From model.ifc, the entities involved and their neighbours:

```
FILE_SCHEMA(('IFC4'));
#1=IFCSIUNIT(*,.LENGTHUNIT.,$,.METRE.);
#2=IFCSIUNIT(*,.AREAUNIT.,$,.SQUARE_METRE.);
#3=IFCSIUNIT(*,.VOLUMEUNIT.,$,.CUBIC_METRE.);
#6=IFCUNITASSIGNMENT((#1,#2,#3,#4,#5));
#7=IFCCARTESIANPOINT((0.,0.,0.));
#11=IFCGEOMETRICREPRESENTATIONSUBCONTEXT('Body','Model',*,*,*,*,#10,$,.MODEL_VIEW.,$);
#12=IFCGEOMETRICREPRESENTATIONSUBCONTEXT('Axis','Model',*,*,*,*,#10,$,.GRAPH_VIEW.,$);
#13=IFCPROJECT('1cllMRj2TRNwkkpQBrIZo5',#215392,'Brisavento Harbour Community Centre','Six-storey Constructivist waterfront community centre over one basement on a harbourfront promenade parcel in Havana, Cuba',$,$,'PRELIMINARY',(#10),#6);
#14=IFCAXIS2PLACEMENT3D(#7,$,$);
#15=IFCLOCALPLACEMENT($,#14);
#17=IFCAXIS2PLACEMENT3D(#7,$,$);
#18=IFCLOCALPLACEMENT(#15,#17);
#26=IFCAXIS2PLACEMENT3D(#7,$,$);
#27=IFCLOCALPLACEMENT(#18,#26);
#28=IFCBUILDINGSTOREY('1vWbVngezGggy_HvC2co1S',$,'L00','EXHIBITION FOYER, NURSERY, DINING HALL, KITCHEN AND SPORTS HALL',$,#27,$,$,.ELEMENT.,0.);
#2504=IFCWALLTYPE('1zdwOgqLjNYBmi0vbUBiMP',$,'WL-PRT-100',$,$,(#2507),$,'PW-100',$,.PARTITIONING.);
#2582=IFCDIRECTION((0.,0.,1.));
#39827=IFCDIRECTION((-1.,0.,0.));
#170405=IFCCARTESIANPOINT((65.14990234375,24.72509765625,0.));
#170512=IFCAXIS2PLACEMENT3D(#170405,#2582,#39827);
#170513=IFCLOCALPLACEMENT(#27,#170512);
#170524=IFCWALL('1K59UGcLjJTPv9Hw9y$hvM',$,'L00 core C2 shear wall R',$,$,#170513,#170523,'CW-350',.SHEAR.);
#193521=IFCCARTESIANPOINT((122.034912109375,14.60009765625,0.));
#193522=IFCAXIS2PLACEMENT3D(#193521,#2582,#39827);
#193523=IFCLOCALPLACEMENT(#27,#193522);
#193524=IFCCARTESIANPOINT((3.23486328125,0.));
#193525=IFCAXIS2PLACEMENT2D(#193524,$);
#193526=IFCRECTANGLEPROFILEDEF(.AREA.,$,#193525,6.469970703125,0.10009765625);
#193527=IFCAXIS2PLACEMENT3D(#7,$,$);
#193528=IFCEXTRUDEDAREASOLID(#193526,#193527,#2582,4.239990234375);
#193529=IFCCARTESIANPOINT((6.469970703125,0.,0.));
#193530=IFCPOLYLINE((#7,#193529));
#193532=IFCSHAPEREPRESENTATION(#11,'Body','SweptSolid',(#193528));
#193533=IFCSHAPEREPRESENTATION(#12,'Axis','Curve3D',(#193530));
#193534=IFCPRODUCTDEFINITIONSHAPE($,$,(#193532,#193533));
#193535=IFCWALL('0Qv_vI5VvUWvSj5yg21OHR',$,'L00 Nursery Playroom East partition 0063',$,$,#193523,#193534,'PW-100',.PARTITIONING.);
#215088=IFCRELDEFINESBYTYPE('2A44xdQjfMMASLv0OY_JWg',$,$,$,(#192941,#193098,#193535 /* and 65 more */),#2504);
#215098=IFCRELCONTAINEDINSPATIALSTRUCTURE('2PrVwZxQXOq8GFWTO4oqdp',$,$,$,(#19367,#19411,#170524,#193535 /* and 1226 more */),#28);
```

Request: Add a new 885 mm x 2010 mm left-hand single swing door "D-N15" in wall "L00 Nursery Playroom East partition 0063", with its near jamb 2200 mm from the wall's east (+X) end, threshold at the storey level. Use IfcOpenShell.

```python
import numpy as np
import ifcopenshell
import ifcopenshell.api.feature
import ifcopenshell.api.geometry
import ifcopenshell.api.root
import ifcopenshell.api.spatial
import ifcopenshell.geom
import ifcopenshell.util.element
import ifcopenshell.util.placement
import ifcopenshell.util.representation
import ifcopenshell.util.shape
import ifcopenshell.util.unit

model = ifcopenshell.open("model.ifc")
unit_scale = ifcopenshell.util.unit.calculate_unit_scale(model)
settings = ifcopenshell.geom.settings()


def volume(element):
    """Net volume in cubic metres, openings subtracted."""
    shape = ifcopenshell.geom.create_shape(settings, element)
    return ifcopenshell.util.shape.get_volume(shape.geometry)


wall = model.by_id(193535)
storey = ifcopenshell.util.element.get_container(wall, ifc_class="IfcBuildingStorey")
context = ifcopenshell.util.representation.get_context(model, "Model", "Body", "MODEL_VIEW")
before = volume(wall)

width, height, from_end, sill = 0.885, 2.01, 2.2, 0.0  # metres

# The wall runs along its own X axis, and the end named is its -X end.
wall_shape = ifcopenshell.geom.create_shape(settings, wall)
x, y, z = ifcopenshell.util.shape.get_vertices(wall_shape.geometry).T
start = x.min() + from_end
face, thickness = float(y.min()), float(y.max() - y.min())
wall_matrix = ifcopenshell.util.placement.get_local_placement(wall.ObjectPlacement)
level = ifcopenshell.util.placement.get_local_placement(storey.ObjectPlacement)[2, 3]


def in_wall(x, y):
    """Placement at x, y metres in the wall's axes, at sill height."""
    matrix = wall_matrix.copy()
    matrix[:, 3] = wall_matrix @ np.array([x / unit_scale, y / unit_scale, 0.0, 1.0])
    matrix[2, 3] = level + sill / unit_scale
    return matrix


# Opening: a box that overshoots both wall faces by 50 mm.
opening = ifcopenshell.api.root.create_entity(model, ifc_class="IfcOpeningElement", predefined_type="OPENING")
box = ifcopenshell.api.geometry.add_wall_representation(
    model, context=context, length=width, height=height, thickness=thickness + 0.1
)
ifcopenshell.api.geometry.assign_representation(model, product=opening, representation=box)
ifcopenshell.api.geometry.edit_object_placement(model, product=opening, matrix=in_wall(start, face - 0.05), is_si=False)
ifcopenshell.api.feature.add_feature(model, feature=opening, element=wall)

door = ifcopenshell.api.root.create_entity(model, ifc_class="IfcDoor", name="D-N15", predefined_type="DOOR")
door.OverallWidth, door.OverallHeight = width / unit_scale, height / unit_scale
door.OperationType = "SINGLE_SWING_LEFT"
body = ifcopenshell.api.geometry.add_door_representation(
    model,
    context=context,
    overall_width=door.OverallWidth,
    overall_height=door.OverallHeight,
    operation_type="SINGLE_SWING_LEFT",
    lining_properties={"LiningDepth": thickness / unit_scale, "ThresholdDepth": thickness / unit_scale},
)
ifcopenshell.api.geometry.assign_representation(model, product=door, representation=body)
ifcopenshell.api.spatial.assign_container(model, products=[door], relating_structure=storey)
ifcopenshell.api.feature.add_filling(model, opening=opening, element=door)

# The lining spans the wall, so the door starts at the wall face.
ifcopenshell.api.geometry.edit_object_placement(model, product=door, matrix=in_wall(start, face), is_si=False)

after = volume(wall)

print(f"wall volume {before:.3f} -> {after:.3f} m3")

model.write("model_rev.ifc")
```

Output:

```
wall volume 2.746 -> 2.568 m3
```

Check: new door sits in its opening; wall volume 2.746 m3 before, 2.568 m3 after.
